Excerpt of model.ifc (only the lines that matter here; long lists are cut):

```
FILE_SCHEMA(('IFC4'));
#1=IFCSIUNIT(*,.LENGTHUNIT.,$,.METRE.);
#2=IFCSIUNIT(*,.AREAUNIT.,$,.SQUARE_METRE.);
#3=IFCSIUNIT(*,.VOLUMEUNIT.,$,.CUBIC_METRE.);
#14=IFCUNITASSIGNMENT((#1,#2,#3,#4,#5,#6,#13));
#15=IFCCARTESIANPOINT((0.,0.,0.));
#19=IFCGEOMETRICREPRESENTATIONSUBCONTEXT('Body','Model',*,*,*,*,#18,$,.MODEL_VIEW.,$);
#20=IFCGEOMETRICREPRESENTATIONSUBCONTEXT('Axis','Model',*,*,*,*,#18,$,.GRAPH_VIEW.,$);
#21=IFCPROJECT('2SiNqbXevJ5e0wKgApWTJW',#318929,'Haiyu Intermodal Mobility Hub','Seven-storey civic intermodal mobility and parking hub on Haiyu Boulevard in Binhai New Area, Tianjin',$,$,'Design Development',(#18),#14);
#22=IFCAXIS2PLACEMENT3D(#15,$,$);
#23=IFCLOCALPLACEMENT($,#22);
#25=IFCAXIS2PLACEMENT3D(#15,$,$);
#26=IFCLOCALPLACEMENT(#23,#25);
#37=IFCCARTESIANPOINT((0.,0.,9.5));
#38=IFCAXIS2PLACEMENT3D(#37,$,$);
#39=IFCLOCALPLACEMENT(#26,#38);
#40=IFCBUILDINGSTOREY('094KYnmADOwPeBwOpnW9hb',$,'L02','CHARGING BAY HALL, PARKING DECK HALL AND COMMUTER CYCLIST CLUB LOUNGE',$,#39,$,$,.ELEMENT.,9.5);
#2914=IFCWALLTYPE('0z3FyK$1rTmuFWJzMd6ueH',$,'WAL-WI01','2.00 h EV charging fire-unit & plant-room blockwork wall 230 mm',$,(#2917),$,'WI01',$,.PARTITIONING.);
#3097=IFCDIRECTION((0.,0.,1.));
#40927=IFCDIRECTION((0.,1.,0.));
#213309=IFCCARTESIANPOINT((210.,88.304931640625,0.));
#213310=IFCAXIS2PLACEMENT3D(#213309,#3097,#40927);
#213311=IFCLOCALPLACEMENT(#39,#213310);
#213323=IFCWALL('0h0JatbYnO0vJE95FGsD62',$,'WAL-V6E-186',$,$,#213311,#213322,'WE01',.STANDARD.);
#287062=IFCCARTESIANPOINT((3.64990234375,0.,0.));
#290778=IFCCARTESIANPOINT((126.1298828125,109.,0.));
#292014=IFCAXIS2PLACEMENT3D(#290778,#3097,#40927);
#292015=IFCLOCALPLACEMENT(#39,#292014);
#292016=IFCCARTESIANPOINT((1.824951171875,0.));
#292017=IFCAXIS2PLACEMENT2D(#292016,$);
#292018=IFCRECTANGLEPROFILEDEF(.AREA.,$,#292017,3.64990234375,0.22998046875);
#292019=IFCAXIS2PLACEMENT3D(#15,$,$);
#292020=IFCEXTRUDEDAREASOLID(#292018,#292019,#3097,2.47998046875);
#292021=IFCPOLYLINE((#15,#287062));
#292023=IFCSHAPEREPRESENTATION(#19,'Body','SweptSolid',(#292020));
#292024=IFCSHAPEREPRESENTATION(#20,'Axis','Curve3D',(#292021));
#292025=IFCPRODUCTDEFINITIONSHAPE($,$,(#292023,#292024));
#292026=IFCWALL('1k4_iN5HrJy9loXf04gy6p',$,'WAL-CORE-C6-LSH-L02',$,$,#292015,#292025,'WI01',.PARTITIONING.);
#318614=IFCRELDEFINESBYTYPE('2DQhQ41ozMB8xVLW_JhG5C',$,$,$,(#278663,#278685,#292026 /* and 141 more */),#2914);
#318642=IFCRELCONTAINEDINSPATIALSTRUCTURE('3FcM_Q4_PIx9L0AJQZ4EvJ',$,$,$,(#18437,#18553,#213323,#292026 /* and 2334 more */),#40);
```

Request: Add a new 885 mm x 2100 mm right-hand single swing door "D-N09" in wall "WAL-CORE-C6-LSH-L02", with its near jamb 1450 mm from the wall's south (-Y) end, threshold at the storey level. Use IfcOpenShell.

```python
import numpy as np
import ifcopenshell
import ifcopenshell.api.feature
import ifcopenshell.api.geometry
import ifcopenshell.api.root
import ifcopenshell.api.spatial
import ifcopenshell.geom
import ifcopenshell.util.element
import ifcopenshell.util.placement
import ifcopenshell.util.representation
import ifcopenshell.util.shape
import ifcopenshell.util.unit

model = ifcopenshell.open("model.ifc")
unit_scale = ifcopenshell.util.unit.calculate_unit_scale(model)
settings = ifcopenshell.geom.settings()


def volume(element):
    """Net volume in cubic metres, openings subtracted."""
    shape = ifcopenshell.geom.create_shape(settings, element)
    return ifcopenshell.util.shape.get_volume(shape.geometry)


wall = model.by_id(292026)
storey = ifcopenshell.util.element.get_container(wall, ifc_class="IfcBuildingStorey")
context = ifcopenshell.util.representation.get_context(model, "Model", "Body", "MODEL_VIEW")
before = volume(wall)

width, height, from_end, sill = 0.885, 2.1, 1.45, 0.0  # metres

# The wall runs along its own X axis, and the end named is its -X end.
wall_shape = ifcopenshell.geom.create_shape(settings, wall)
x, y, z = ifcopenshell.util.shape.get_vertices(wall_shape.geometry).T
start = x.min() + from_end
face, thickness = float(y.min()), float(y.max() - y.min())
wall_matrix = ifcopenshell.util.placement.get_local_placement(wall.ObjectPlacement)
level = ifcopenshell.util.placement.get_local_placement(storey.ObjectPlacement)[2, 3]


def in_wall(x, y):
    """Placement at x, y metres in the wall's axes, at sill height."""
    matrix = wall_matrix.copy()
    matrix[:, 3] = wall_matrix @ np.array([x / unit_scale, y / unit_scale, 0.0, 1.0])
    matrix[2, 3] = level + sill / unit_scale
    return matrix


# Opening: a box that overshoots both wall faces by 50 mm.
opening = ifcopenshell.api.root.create_entity(model, ifc_class="IfcOpeningElement", predefined_type="OPENING")
box = ifcopenshell.api.geometry.add_wall_representation(
    model, context=context, length=width, height=height, thickness=thickness + 0.1
)
ifcopenshell.api.geometry.assign_representation(model, product=opening, representation=box)
ifcopenshell.api.geometry.edit_object_placement(model, product=opening, matrix=in_wall(start, face - 0.05), is_si=False)
ifcopenshell.api.feature.add_feature(model, feature=opening, element=wall)

door = ifcopenshell.api.root.create_entity(model, ifc_class="IfcDoor", name="D-N09", predefined_type="DOOR")
door.OverallWidth, door.OverallHeight = width / unit_scale, height / unit_scale
door.OperationType = "SINGLE_SWING_RIGHT"
body = ifcopenshell.api.geometry.add_door_representation(
    model,
    context=context,
    overall_width=door.OverallWidth,
    overall_height=door.OverallHeight,
    operation_type="SINGLE_SWING_RIGHT",
    lining_properties={"LiningDepth": thickness / unit_scale, "ThresholdDepth": thickness / unit_scale},
)
ifcopenshell.api.geometry.assign_representation(model, product=door, representation=body)
ifcopenshell.api.spatial.assign_container(model, products=[door], relating_structure=storey)
ifcopenshell.api.feature.add_filling(model, opening=opening, element=door)

# The lining spans the wall, so the door starts at the wall face.
ifcopenshell.api.geometry.edit_object_placement(model, product=door, matrix=in_wall(start, face), is_si=False)

after = volume(wall)

print(f"wall volume {before:.3f} -> {after:.3f} m3")

model.write("model-out.ifc")
```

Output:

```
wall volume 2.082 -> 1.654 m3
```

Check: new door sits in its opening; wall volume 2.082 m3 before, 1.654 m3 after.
